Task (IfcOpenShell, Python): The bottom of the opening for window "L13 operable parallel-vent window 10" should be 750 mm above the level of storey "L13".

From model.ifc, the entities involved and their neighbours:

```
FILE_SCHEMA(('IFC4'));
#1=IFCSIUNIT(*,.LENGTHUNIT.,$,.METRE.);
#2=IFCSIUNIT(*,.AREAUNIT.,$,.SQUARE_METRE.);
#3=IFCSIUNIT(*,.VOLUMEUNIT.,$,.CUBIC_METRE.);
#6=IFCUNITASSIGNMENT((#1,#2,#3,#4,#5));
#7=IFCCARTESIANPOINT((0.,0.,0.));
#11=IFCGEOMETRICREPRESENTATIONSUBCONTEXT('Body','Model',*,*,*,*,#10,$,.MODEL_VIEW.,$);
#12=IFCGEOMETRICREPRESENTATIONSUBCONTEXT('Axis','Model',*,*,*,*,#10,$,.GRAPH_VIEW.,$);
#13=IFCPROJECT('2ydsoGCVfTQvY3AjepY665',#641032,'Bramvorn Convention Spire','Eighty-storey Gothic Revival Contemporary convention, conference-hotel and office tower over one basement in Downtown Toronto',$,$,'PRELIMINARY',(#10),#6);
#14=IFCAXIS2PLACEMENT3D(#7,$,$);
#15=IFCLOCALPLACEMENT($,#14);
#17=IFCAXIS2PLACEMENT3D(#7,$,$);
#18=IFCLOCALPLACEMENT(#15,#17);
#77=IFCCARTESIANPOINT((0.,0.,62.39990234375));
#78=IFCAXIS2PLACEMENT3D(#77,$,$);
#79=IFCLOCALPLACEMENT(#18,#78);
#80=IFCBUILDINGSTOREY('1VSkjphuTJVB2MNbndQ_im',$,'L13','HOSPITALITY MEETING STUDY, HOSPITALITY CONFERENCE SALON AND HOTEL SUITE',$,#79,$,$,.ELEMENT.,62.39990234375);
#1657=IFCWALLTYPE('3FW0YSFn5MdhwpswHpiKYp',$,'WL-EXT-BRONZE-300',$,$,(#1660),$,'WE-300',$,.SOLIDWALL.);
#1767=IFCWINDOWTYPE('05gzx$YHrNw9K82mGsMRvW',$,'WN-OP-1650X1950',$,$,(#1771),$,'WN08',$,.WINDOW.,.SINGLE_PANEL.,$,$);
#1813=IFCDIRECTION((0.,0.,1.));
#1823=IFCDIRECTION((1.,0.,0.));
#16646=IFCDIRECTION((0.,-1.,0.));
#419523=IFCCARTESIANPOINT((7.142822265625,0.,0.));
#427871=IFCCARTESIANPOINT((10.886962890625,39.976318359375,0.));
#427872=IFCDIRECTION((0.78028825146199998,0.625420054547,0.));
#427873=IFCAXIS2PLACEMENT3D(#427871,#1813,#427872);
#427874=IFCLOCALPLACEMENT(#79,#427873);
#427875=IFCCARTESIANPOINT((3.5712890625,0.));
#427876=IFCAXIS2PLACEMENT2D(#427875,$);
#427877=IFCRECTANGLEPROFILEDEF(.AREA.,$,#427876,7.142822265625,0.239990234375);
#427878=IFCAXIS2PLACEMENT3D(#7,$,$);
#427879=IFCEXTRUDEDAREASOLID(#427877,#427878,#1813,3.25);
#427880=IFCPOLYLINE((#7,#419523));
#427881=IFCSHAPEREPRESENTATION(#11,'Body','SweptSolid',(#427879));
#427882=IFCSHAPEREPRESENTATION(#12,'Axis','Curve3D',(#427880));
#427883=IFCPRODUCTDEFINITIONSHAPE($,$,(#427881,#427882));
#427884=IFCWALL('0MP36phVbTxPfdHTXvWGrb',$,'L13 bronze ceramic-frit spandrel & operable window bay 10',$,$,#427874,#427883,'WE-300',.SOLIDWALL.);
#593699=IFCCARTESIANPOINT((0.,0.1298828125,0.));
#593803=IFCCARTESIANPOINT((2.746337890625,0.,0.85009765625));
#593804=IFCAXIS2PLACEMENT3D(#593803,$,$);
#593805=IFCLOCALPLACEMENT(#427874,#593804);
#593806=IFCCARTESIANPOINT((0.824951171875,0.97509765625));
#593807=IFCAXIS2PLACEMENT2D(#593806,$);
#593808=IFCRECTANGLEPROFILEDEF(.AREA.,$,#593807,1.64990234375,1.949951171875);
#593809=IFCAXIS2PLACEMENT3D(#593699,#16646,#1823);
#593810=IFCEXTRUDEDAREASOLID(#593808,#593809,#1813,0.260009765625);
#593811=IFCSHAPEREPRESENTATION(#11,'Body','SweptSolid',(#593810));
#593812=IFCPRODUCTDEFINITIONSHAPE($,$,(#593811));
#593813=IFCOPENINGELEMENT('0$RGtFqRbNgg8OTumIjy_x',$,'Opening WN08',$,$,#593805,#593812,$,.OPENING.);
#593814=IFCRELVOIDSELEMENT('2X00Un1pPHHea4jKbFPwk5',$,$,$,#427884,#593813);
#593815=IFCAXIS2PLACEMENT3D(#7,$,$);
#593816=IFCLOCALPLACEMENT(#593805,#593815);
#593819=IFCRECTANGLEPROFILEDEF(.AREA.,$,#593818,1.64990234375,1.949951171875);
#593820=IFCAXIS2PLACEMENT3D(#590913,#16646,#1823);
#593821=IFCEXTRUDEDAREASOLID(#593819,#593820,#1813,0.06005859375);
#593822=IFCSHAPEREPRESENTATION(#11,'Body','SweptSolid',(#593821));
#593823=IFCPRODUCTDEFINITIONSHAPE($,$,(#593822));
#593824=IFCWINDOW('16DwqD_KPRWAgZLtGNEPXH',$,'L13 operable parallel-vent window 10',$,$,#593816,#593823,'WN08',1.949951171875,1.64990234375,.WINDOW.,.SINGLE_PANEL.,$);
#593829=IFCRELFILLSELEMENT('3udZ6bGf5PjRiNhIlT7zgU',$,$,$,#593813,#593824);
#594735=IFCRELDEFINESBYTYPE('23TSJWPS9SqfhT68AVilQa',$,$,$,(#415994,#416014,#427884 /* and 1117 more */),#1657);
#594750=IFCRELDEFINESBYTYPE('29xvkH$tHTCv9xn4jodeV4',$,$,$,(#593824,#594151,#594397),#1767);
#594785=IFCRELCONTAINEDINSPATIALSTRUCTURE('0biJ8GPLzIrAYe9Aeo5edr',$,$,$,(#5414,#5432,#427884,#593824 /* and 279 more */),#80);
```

```python
import numpy as np
import ifcopenshell
import ifcopenshell.api.geometry
import ifcopenshell.geom
import ifcopenshell.util.element
import ifcopenshell.util.placement
import ifcopenshell.util.shape
import ifcopenshell.util.unit

model = ifcopenshell.open("model.ifc")
unit_scale = ifcopenshell.util.unit.calculate_unit_scale(model)

window = model.by_guid("16DwqD_KPRWAgZLtGNEPXH")
opening = window.FillsVoids[0].RelatingOpeningElement
storey = ifcopenshell.util.element.get_container(window, ifc_class="IfcBuildingStorey")
level = ifcopenshell.util.placement.get_local_placement(storey.ObjectPlacement)[2, 3]

# The opening's origin need not be at the sill, so measure its lowest point.
shape = ifcopenshell.geom.create_shape(ifcopenshell.geom.settings(), opening)
bottom = ifcopenshell.util.shape.get_shape_bottom_elevation(shape, shape.geometry) / unit_scale
dz = level + 0.75 / unit_scale - bottom

shift = np.array([0.0, 0.0, dz])
# The window is placed relative to its opening, so it follows when the opening moves.
matrix = ifcopenshell.util.placement.get_local_placement(opening.ObjectPlacement)
matrix[:3, 3] += shift
ifcopenshell.api.geometry.edit_object_placement(
    model, product=opening, matrix=matrix, is_si=False, should_transform_children=True
)

print(f"moved by {dz * unit_scale:+.3f} m")

model.write("model-out.ifc")
```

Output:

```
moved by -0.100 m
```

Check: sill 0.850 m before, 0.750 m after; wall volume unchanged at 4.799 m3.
